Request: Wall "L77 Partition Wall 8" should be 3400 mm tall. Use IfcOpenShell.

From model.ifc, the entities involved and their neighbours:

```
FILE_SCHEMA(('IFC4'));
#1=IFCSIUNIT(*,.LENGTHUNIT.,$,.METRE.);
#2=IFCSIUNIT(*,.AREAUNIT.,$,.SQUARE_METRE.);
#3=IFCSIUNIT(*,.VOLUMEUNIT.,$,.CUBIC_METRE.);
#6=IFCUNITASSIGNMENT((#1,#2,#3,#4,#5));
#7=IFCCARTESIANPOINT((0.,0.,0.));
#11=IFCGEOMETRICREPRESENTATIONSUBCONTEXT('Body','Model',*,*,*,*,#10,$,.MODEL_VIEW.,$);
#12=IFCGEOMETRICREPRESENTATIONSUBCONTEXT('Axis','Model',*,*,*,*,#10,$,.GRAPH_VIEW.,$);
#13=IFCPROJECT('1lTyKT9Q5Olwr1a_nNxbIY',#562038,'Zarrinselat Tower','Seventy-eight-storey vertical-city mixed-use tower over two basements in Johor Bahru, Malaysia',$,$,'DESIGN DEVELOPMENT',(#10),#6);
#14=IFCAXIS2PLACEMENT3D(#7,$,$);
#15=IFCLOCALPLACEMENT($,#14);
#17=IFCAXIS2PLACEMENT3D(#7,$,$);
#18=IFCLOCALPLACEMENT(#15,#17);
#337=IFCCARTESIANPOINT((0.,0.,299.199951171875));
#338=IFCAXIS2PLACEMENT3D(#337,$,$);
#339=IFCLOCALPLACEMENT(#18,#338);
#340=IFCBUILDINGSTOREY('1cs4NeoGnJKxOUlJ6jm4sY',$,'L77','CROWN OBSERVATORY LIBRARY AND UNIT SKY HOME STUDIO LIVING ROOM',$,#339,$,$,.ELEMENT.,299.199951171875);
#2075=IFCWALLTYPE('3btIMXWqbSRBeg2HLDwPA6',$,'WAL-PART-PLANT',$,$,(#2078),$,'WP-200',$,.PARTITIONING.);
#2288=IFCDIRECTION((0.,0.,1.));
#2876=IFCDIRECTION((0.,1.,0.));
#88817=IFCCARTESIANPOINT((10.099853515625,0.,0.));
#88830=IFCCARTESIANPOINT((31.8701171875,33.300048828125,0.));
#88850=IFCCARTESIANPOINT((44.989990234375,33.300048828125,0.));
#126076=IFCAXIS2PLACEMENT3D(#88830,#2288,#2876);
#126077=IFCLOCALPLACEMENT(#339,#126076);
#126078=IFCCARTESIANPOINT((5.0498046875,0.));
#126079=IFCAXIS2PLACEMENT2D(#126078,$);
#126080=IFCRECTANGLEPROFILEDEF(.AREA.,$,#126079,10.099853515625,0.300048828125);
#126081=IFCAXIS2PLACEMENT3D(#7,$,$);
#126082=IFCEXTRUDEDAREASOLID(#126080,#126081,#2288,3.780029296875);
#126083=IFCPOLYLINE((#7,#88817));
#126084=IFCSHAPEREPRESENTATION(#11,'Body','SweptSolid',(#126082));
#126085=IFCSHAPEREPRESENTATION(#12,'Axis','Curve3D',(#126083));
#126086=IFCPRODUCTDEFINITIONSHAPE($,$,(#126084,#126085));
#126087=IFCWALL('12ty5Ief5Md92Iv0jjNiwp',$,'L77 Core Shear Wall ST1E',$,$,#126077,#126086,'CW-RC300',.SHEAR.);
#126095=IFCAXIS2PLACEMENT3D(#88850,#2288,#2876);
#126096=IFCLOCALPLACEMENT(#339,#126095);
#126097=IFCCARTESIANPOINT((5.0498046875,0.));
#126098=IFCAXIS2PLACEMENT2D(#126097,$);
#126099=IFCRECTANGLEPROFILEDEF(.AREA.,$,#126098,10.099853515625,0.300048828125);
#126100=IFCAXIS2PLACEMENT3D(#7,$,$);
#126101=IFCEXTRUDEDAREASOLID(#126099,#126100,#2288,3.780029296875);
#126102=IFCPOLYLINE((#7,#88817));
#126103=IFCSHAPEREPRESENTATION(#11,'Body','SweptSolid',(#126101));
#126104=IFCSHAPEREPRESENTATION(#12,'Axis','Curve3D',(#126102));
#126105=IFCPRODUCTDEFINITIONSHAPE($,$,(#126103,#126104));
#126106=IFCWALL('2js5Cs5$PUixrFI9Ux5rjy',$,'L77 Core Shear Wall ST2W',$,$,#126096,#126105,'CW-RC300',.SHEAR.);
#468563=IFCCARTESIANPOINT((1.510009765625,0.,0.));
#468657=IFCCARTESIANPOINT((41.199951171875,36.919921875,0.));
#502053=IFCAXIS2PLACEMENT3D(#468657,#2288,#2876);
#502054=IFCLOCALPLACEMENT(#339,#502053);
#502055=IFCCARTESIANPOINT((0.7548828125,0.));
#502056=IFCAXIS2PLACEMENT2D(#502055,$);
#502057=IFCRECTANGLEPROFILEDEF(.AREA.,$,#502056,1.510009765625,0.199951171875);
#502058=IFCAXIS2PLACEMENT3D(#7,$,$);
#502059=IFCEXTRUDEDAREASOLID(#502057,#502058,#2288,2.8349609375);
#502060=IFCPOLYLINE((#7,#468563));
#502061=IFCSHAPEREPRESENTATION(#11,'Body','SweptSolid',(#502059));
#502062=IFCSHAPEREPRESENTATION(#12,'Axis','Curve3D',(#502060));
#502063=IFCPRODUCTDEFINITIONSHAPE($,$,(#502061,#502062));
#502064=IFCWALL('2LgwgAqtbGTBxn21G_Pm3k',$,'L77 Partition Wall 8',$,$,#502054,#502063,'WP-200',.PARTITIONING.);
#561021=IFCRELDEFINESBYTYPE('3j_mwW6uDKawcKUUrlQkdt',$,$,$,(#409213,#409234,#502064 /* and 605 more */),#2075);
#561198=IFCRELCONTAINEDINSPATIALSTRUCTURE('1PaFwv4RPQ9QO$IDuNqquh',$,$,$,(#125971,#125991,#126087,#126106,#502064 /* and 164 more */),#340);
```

```python
import ifcopenshell
import ifcopenshell.geom
import ifcopenshell.util.representation
import ifcopenshell.util.shape

model = ifcopenshell.open("model.ifc")
settings = ifcopenshell.geom.settings()


def volume(element):
    """Net volume in cubic metres, openings subtracted."""
    shape = ifcopenshell.geom.create_shape(settings, element)
    return ifcopenshell.util.shape.get_volume(shape.geometry)


wall = model.by_guid("2LgwgAqtbGTBxn21G_Pm3k")
before = volume(wall)

body = ifcopenshell.util.representation.get_representation(wall, "Model", "Body")
solid = body.Items[0]
old_height = solid.Depth
solid.Depth = 3.4
after = volume(wall)

print(f"height {old_height:g} -> {solid.Depth:g}, volume {before:.3f} -> {after:.3f} m3")

model.write("model_v2.ifc")
```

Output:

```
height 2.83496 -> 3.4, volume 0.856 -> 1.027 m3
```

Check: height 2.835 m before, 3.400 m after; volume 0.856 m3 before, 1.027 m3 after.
